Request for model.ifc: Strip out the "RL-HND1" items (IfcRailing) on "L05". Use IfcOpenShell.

First a look at what the model holds.

```python
import ifcopenshell
import ifcopenshell.util.element

model = ifcopenshell.open("model.ifc")
print(model.schema)
storey = next(s for s in model.by_type("IfcBuildingStorey") if s.Name == "L05")
railings = [e for e in ifcopenshell.util.element.get_decomposition(storey) if e.is_a("IfcRailing")]
seen = {}
for e in railings:
    element_type = ifcopenshell.util.element.get_type(e)
    name = element_type.Name if element_type not in (None, e) else None
    seen[name] = seen.get(name, 0) + 1
for name, count in sorted(seen.items(), key=str):
    print(count, "x", name)
```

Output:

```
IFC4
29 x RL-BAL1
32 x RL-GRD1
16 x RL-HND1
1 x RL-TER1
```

```python
import ifcopenshell
import ifcopenshell.api.root
import ifcopenshell.util.element

model = ifcopenshell.open("model.ifc")

storey = next(s for s in model.by_type("IfcBuildingStorey") if s.Name == "L05")
railings = [e for e in ifcopenshell.util.element.get_decomposition(storey) if e.is_a("IfcRailing")]
targets = [e for e in railings if (t := ifcopenshell.util.element.get_type(e)) not in (None, e) and t.Name == "RL-HND1"]

for e in targets:
    ifcopenshell.api.root.remove_product(model, product=e)
print(len(targets), "removed")

model.write("model-out.ifc")
```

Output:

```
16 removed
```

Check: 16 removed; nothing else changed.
